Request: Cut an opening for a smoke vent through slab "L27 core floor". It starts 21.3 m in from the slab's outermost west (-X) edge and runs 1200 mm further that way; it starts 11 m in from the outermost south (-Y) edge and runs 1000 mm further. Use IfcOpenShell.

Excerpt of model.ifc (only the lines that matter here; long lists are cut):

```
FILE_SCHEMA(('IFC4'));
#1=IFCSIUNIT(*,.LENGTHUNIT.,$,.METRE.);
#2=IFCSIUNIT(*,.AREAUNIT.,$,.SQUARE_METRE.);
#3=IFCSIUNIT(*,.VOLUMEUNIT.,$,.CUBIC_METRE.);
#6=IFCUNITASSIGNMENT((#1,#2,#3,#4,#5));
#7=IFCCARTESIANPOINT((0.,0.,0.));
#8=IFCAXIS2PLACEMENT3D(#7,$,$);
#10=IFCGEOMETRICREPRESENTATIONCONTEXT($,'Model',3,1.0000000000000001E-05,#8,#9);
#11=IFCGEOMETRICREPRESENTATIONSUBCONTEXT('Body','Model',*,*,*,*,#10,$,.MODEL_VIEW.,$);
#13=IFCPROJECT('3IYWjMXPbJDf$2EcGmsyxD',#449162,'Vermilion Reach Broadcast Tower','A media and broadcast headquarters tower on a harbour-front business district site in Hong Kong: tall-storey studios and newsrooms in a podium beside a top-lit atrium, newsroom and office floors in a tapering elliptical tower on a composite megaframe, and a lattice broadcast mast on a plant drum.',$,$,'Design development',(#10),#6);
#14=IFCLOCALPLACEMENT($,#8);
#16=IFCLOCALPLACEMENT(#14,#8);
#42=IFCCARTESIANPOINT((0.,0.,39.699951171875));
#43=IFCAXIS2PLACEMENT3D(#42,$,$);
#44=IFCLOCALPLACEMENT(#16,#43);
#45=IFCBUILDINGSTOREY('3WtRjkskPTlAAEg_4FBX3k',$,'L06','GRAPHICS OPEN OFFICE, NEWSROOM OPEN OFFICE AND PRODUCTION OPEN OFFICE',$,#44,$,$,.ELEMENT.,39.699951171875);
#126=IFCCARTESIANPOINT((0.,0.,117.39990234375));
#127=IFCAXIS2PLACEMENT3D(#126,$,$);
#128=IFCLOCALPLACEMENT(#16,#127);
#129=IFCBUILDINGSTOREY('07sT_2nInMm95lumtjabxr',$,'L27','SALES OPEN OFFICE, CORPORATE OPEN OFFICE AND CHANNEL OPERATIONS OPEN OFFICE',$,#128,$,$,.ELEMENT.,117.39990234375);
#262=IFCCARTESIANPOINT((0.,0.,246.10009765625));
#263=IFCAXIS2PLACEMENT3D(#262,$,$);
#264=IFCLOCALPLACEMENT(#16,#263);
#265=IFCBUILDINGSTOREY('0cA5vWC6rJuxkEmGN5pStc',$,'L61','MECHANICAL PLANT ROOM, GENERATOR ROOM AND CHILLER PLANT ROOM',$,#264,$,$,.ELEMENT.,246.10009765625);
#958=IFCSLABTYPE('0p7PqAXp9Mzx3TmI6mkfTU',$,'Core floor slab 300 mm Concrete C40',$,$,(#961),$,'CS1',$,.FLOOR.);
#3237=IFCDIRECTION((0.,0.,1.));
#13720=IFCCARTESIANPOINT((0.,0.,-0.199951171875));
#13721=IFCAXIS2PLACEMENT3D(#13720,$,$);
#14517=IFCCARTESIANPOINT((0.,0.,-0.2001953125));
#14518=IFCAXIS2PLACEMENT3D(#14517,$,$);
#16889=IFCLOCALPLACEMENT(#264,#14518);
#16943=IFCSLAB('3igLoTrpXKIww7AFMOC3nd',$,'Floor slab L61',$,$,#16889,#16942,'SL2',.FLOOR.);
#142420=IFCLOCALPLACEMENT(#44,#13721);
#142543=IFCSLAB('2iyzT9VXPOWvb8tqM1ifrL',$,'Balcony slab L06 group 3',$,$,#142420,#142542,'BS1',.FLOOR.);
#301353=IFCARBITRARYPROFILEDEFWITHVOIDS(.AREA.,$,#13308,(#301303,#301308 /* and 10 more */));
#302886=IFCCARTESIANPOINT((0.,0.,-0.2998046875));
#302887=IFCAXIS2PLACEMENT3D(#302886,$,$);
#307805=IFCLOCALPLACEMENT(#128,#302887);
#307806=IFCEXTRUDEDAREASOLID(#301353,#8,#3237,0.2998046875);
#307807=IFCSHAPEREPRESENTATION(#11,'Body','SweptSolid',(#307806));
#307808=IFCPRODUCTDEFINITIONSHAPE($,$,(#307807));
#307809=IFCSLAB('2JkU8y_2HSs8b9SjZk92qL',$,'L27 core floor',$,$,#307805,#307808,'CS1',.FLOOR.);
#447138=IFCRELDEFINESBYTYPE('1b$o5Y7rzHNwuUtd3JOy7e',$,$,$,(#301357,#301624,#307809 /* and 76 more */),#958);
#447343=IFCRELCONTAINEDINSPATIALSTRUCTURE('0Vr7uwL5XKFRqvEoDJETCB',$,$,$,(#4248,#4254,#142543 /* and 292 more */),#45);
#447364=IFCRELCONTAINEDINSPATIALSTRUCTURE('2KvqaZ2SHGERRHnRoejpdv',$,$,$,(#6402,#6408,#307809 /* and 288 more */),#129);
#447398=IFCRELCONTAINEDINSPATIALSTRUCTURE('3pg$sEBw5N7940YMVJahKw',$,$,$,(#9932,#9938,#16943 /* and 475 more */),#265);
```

```python
import numpy as np
import ifcopenshell
import ifcopenshell.api.feature
import ifcopenshell.api.geometry
import ifcopenshell.api.root
import ifcopenshell.geom
import ifcopenshell.util.placement
import ifcopenshell.util.representation
import ifcopenshell.util.shape
import ifcopenshell.util.unit

model = ifcopenshell.open("model.ifc")
unit_scale = ifcopenshell.util.unit.calculate_unit_scale(model)
settings = ifcopenshell.geom.settings()


def volume(element):
    """Net volume in cubic metres, openings subtracted."""
    shape = ifcopenshell.geom.create_shape(settings, element)
    return ifcopenshell.util.shape.get_volume(shape.geometry)


slab = model.by_guid("2JkU8y_2HSs8b9SjZk92qL")
before = volume(slab)

# Extent in the slab's own axes, in metres. The edges named are its -X and -Y sides.
slab_shape = ifcopenshell.geom.create_shape(settings, slab)
vertices = ifcopenshell.util.shape.get_vertices(slab_shape.geometry)
x_min, y_min, bottom = vertices.min(axis=0)
top = vertices[:, 2].max()

opening = ifcopenshell.api.root.create_entity(model, ifc_class="IfcOpeningElement", name="Smoke vent opening", predefined_type="OPENING")
context = ifcopenshell.util.representation.get_context(model, "Model", "Body", "MODEL_VIEW")
width, depth = 1.2, 1
outline = [(0.0, 0.0), (width, 0.0), (width, depth), (0.0, depth), (0.0, 0.0)]
# Overshoot both faces by 50 mm so the cut is clean.
shape = ifcopenshell.api.geometry.add_slab_representation(
    model, context=context, depth=top - bottom + 0.1, polyline=outline
)
ifcopenshell.api.geometry.assign_representation(model, product=opening, representation=shape)

matrix = ifcopenshell.util.placement.get_local_placement(slab.ObjectPlacement)
matrix[:, 3] = matrix @ np.append(np.array([x_min + 21.3, y_min + 11, bottom - 0.05]) / unit_scale, 1.0)
ifcopenshell.api.geometry.edit_object_placement(model, product=opening, matrix=matrix, is_si=False)
ifcopenshell.api.feature.add_feature(model, feature=opening, element=slab)

after = volume(slab)

print(f"slab volume {before:.3f} -> {after:.3f} m3")

model.write("model-out.ifc")
```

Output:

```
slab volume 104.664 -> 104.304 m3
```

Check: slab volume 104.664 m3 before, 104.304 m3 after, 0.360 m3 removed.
